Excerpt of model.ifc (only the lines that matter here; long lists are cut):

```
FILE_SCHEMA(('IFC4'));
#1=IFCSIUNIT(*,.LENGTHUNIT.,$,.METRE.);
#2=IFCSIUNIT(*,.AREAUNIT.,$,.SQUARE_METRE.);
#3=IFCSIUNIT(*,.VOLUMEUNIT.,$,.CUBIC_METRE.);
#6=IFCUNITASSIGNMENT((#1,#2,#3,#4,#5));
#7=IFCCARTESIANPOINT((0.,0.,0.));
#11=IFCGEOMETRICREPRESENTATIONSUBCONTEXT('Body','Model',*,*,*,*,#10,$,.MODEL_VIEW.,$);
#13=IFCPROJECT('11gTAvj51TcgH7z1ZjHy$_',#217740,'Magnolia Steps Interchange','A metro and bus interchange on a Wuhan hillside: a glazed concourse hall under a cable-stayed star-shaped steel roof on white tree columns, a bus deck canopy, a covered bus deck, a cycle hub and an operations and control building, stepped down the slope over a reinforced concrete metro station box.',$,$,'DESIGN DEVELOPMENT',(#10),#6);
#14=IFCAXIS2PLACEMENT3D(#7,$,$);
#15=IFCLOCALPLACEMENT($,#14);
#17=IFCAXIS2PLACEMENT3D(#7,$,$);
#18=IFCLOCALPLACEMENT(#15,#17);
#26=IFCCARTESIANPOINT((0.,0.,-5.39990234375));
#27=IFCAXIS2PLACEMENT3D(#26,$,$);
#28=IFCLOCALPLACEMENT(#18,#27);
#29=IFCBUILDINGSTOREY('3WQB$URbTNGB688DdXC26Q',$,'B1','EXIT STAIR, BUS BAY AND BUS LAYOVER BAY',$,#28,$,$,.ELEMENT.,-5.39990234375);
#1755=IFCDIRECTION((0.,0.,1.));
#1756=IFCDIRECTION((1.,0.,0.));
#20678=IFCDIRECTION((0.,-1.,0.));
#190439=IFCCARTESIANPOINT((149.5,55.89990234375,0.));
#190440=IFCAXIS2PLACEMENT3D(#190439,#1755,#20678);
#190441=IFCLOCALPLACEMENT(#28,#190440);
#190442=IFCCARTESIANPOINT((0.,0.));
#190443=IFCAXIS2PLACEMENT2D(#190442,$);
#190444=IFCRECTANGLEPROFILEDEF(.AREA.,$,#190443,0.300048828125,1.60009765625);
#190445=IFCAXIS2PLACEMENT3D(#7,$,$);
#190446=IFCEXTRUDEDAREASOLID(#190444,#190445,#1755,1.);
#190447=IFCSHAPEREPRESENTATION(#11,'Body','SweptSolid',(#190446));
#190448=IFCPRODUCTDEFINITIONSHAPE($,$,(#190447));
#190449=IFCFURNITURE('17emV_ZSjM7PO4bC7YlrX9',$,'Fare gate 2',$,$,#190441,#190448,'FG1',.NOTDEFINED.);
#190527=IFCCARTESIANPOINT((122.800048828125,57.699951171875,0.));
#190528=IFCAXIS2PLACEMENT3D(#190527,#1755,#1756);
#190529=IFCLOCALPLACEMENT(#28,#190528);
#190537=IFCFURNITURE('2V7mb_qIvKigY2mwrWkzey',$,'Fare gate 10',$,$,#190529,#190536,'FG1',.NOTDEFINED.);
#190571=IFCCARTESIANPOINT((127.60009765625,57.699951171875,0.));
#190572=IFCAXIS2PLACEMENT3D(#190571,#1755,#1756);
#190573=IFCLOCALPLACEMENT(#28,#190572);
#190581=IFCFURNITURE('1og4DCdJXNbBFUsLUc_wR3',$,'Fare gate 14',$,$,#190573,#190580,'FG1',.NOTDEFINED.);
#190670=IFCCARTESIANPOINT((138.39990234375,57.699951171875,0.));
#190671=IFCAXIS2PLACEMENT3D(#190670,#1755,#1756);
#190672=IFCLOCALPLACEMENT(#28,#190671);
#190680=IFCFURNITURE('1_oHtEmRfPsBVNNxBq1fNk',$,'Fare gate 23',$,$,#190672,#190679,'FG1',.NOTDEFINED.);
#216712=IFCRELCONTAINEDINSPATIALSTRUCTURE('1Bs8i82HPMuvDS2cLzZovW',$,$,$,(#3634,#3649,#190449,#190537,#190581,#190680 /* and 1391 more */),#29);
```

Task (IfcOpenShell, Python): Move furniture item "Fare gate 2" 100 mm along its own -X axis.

```python
import ifcopenshell
import ifcopenshell.api.geometry
import ifcopenshell.util.placement

model = ifcopenshell.open("model.ifc")

item = model.by_id(190449)
matrix = ifcopenshell.util.placement.get_local_placement(item.ObjectPlacement)
matrix[:3, 3] -= matrix[:3, 0] * 0.1
ifcopenshell.api.geometry.edit_object_placement(model, product=item, matrix=matrix, is_si=False)

print(ifcopenshell.util.placement.get_local_placement(item.ObjectPlacement).round(3) + 0.0)

model.write("model-out.ifc")
```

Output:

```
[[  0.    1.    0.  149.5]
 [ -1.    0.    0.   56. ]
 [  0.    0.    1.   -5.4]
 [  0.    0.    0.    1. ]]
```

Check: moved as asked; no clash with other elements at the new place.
